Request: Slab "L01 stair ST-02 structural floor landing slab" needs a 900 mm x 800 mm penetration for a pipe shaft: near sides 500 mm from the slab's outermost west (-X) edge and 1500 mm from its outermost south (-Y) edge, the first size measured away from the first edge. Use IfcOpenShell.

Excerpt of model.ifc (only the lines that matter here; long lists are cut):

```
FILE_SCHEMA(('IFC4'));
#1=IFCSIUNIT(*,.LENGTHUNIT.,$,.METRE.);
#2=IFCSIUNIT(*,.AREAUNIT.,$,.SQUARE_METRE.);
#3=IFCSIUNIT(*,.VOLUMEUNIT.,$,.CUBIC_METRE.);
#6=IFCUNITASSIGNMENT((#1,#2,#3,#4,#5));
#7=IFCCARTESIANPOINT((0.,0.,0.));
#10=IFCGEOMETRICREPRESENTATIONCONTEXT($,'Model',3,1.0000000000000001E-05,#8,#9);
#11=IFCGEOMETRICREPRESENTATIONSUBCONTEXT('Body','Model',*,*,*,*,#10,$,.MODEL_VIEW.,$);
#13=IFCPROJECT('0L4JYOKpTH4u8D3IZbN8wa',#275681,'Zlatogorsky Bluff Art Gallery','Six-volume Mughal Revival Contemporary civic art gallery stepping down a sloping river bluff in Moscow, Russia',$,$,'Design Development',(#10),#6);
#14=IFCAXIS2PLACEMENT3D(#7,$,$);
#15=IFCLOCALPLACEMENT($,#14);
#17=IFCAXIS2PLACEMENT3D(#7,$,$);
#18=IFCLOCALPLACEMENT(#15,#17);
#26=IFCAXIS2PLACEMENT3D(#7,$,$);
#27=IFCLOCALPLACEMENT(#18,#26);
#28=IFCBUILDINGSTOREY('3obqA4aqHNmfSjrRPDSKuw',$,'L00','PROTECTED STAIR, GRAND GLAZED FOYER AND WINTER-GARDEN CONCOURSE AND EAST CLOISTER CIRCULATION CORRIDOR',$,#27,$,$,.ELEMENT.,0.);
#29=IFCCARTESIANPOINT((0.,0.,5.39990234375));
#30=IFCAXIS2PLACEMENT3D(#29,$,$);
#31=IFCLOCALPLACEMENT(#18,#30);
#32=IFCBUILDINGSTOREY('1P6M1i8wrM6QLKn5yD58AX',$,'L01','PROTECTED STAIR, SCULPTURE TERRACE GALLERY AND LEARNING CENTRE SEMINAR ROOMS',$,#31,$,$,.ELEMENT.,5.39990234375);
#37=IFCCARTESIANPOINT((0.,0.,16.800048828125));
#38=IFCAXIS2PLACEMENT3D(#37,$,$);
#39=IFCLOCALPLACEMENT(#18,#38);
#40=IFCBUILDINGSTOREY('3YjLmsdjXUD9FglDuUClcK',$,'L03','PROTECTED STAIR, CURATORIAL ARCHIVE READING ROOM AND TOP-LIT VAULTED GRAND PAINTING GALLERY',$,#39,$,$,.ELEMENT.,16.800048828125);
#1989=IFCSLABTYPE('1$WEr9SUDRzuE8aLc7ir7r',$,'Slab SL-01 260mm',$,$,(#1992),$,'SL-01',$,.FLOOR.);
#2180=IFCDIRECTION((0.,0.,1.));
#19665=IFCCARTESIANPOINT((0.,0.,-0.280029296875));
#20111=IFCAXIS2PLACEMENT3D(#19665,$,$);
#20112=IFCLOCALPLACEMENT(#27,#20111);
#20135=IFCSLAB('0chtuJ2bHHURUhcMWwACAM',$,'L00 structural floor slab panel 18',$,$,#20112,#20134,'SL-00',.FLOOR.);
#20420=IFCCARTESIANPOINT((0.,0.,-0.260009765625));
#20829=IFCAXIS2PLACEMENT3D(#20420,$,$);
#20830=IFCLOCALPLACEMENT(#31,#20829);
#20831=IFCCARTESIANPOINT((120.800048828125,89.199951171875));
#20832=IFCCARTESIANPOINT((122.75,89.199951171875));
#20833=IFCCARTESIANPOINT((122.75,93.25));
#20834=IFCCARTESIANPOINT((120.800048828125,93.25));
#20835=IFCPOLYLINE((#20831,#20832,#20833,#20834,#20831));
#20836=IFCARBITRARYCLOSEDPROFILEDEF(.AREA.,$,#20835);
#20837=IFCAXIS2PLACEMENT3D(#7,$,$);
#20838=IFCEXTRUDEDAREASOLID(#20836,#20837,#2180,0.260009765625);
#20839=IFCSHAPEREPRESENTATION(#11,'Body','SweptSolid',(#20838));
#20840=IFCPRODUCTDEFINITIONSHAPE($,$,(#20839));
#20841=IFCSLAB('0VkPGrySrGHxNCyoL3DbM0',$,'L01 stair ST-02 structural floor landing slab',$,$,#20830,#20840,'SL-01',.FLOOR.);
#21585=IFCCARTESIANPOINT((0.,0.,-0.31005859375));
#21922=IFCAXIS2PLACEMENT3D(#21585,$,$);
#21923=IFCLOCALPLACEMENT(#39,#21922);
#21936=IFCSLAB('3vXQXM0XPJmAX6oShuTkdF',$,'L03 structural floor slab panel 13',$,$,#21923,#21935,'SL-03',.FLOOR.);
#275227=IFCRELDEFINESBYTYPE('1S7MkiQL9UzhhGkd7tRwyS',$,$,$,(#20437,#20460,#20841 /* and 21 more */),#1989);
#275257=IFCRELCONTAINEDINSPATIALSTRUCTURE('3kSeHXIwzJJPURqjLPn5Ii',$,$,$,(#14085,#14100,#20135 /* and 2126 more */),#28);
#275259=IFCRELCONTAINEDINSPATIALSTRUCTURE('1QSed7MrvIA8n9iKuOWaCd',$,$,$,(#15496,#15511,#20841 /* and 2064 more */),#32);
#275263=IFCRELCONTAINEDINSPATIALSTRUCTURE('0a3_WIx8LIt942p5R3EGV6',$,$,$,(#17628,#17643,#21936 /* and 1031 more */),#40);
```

```python
import numpy as np
import ifcopenshell
import ifcopenshell.api.feature
import ifcopenshell.api.geometry
import ifcopenshell.api.root
import ifcopenshell.geom
import ifcopenshell.util.placement
import ifcopenshell.util.representation
import ifcopenshell.util.shape
import ifcopenshell.util.unit

model = ifcopenshell.open("model.ifc")
unit_scale = ifcopenshell.util.unit.calculate_unit_scale(model)
settings = ifcopenshell.geom.settings()


def volume(element):
    """Net volume in cubic metres, openings subtracted."""
    shape = ifcopenshell.geom.create_shape(settings, element)
    return ifcopenshell.util.shape.get_volume(shape.geometry)


slab = model.by_id(20841)
before = volume(slab)

# Extent in the slab's own axes, in metres. The edges named are its -X and -Y sides.
slab_shape = ifcopenshell.geom.create_shape(settings, slab)
vertices = ifcopenshell.util.shape.get_vertices(slab_shape.geometry)
x_min, y_min, bottom = vertices.min(axis=0)
top = vertices[:, 2].max()

opening = ifcopenshell.api.root.create_entity(model, ifc_class="IfcOpeningElement", name="Pipe shaft opening", predefined_type="OPENING")
context = ifcopenshell.util.representation.get_context(model, "Model", "Body", "MODEL_VIEW")
width, depth = 0.9, 0.8
outline = [(0.0, 0.0), (width, 0.0), (width, depth), (0.0, depth), (0.0, 0.0)]
# Overshoot both faces by 50 mm so the cut is clean.
shape = ifcopenshell.api.geometry.add_slab_representation(
    model, context=context, depth=top - bottom + 0.1, polyline=outline
)
ifcopenshell.api.geometry.assign_representation(model, product=opening, representation=shape)

matrix = ifcopenshell.util.placement.get_local_placement(slab.ObjectPlacement)
matrix[:, 3] = matrix @ np.append(np.array([x_min + 0.5, y_min + 1.5, bottom - 0.05]) / unit_scale, 1.0)
ifcopenshell.api.geometry.edit_object_placement(model, product=opening, matrix=matrix, is_si=False)
ifcopenshell.api.feature.add_feature(model, feature=opening, element=slab)

after = volume(slab)

print(f"slab volume {before:.3f} -> {after:.3f} m3")

model.write("model_edited.ifc")
```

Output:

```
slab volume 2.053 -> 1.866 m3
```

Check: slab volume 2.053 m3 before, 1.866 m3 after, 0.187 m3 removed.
